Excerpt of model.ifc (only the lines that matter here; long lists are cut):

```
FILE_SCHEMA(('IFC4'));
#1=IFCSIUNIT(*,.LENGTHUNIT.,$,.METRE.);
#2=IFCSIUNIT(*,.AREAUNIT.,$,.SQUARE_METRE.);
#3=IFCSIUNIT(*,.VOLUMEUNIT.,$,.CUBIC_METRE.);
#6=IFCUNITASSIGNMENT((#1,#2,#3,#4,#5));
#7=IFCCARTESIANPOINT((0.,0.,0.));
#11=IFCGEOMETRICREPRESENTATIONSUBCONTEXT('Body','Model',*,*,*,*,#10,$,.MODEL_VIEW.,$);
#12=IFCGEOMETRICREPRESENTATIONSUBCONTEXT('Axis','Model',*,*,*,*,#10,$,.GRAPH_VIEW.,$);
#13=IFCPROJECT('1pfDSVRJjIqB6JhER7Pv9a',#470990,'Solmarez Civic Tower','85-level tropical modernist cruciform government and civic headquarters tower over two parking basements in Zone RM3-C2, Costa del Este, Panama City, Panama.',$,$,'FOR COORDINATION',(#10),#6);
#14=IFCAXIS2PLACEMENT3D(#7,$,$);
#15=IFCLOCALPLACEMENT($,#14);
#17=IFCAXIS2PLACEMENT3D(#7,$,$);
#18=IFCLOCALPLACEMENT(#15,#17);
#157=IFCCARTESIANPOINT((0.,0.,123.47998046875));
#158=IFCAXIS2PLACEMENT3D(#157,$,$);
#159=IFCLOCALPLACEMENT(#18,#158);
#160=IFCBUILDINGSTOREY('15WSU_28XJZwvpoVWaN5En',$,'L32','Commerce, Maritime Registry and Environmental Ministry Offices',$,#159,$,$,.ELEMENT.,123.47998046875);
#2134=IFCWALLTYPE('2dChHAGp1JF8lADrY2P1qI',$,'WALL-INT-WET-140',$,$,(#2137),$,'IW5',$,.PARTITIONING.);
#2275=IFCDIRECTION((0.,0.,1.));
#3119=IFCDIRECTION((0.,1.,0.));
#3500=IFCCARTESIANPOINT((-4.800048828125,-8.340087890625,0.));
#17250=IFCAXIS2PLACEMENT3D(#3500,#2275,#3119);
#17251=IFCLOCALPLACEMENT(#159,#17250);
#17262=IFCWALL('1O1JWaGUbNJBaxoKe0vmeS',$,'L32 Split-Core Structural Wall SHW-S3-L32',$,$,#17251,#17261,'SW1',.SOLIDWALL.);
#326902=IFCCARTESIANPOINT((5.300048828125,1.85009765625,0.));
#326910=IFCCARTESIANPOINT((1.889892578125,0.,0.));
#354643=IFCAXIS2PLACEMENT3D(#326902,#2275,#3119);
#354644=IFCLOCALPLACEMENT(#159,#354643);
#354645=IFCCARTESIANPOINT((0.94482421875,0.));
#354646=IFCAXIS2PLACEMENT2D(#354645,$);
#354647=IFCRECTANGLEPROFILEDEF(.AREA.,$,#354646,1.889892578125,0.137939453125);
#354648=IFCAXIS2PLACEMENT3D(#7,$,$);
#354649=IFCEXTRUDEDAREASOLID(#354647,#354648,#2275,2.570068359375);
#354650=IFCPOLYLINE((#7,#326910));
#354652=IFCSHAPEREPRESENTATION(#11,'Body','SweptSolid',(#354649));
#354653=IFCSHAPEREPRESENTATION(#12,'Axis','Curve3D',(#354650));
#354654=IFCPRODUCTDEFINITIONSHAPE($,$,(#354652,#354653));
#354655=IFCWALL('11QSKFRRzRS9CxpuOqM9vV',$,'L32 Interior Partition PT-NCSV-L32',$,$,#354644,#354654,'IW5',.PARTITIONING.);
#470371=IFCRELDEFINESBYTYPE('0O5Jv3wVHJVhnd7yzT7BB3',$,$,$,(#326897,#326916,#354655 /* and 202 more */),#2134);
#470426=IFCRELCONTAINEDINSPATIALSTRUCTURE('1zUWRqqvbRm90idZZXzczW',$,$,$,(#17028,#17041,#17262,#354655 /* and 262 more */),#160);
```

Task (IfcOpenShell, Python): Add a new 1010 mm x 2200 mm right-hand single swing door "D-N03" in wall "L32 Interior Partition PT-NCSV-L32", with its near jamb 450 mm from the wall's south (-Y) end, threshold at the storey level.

```python
import numpy as np
import ifcopenshell
import ifcopenshell.api.feature
import ifcopenshell.api.geometry
import ifcopenshell.api.root
import ifcopenshell.api.spatial
import ifcopenshell.geom
import ifcopenshell.util.element
import ifcopenshell.util.placement
import ifcopenshell.util.representation
import ifcopenshell.util.shape
import ifcopenshell.util.unit

model = ifcopenshell.open("model.ifc")
unit_scale = ifcopenshell.util.unit.calculate_unit_scale(model)
settings = ifcopenshell.geom.settings()


def volume(element):
    """Net volume in cubic metres, openings subtracted."""
    shape = ifcopenshell.geom.create_shape(settings, element)
    return ifcopenshell.util.shape.get_volume(shape.geometry)


wall = model.by_guid("11QSKFRRzRS9CxpuOqM9vV")
storey = ifcopenshell.util.element.get_container(wall, ifc_class="IfcBuildingStorey")
context = ifcopenshell.util.representation.get_context(model, "Model", "Body", "MODEL_VIEW")
before = volume(wall)

width, height, from_end, sill = 1.01, 2.2, 0.45, 0.0  # metres

# The wall runs along its own X axis, and the end named is its -X end.
wall_shape = ifcopenshell.geom.create_shape(settings, wall)
x, y, z = ifcopenshell.util.shape.get_vertices(wall_shape.geometry).T
start = x.min() + from_end
face, thickness = float(y.min()), float(y.max() - y.min())
wall_matrix = ifcopenshell.util.placement.get_local_placement(wall.ObjectPlacement)
level = ifcopenshell.util.placement.get_local_placement(storey.ObjectPlacement)[2, 3]


def in_wall(x, y):
    """Placement at x, y metres in the wall's axes, at sill height."""
    matrix = wall_matrix.copy()
    matrix[:, 3] = wall_matrix @ np.array([x / unit_scale, y / unit_scale, 0.0, 1.0])
    matrix[2, 3] = level + sill / unit_scale
    return matrix


# Opening: a box that overshoots both wall faces by 50 mm.
opening = ifcopenshell.api.root.create_entity(model, ifc_class="IfcOpeningElement", predefined_type="OPENING")
box = ifcopenshell.api.geometry.add_wall_representation(
    model, context=context, length=width, height=height, thickness=thickness + 0.1
)
ifcopenshell.api.geometry.assign_representation(model, product=opening, representation=box)
ifcopenshell.api.geometry.edit_object_placement(model, product=opening, matrix=in_wall(start, face - 0.05), is_si=False)
ifcopenshell.api.feature.add_feature(model, feature=opening, element=wall)

door = ifcopenshell.api.root.create_entity(model, ifc_class="IfcDoor", name="D-N03", predefined_type="DOOR")
door.OverallWidth, door.OverallHeight = width / unit_scale, height / unit_scale
door.OperationType = "SINGLE_SWING_RIGHT"
body = ifcopenshell.api.geometry.add_door_representation(
    model,
    context=context,
    overall_width=door.OverallWidth,
    overall_height=door.OverallHeight,
    operation_type="SINGLE_SWING_RIGHT",
    lining_properties={"LiningDepth": thickness / unit_scale, "ThresholdDepth": thickness / unit_scale},
)
ifcopenshell.api.geometry.assign_representation(model, product=door, representation=body)
ifcopenshell.api.spatial.assign_container(model, products=[door], relating_structure=storey)
ifcopenshell.api.feature.add_filling(model, opening=opening, element=door)

# The lining spans the wall, so the door starts at the wall face.
ifcopenshell.api.geometry.edit_object_placement(model, product=door, matrix=in_wall(start, face), is_si=False)

after = volume(wall)

print(f"wall volume {before:.3f} -> {after:.3f} m3")

model.write("model_edited.ifc")
```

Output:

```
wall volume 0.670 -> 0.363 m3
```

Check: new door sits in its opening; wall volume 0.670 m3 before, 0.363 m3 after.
